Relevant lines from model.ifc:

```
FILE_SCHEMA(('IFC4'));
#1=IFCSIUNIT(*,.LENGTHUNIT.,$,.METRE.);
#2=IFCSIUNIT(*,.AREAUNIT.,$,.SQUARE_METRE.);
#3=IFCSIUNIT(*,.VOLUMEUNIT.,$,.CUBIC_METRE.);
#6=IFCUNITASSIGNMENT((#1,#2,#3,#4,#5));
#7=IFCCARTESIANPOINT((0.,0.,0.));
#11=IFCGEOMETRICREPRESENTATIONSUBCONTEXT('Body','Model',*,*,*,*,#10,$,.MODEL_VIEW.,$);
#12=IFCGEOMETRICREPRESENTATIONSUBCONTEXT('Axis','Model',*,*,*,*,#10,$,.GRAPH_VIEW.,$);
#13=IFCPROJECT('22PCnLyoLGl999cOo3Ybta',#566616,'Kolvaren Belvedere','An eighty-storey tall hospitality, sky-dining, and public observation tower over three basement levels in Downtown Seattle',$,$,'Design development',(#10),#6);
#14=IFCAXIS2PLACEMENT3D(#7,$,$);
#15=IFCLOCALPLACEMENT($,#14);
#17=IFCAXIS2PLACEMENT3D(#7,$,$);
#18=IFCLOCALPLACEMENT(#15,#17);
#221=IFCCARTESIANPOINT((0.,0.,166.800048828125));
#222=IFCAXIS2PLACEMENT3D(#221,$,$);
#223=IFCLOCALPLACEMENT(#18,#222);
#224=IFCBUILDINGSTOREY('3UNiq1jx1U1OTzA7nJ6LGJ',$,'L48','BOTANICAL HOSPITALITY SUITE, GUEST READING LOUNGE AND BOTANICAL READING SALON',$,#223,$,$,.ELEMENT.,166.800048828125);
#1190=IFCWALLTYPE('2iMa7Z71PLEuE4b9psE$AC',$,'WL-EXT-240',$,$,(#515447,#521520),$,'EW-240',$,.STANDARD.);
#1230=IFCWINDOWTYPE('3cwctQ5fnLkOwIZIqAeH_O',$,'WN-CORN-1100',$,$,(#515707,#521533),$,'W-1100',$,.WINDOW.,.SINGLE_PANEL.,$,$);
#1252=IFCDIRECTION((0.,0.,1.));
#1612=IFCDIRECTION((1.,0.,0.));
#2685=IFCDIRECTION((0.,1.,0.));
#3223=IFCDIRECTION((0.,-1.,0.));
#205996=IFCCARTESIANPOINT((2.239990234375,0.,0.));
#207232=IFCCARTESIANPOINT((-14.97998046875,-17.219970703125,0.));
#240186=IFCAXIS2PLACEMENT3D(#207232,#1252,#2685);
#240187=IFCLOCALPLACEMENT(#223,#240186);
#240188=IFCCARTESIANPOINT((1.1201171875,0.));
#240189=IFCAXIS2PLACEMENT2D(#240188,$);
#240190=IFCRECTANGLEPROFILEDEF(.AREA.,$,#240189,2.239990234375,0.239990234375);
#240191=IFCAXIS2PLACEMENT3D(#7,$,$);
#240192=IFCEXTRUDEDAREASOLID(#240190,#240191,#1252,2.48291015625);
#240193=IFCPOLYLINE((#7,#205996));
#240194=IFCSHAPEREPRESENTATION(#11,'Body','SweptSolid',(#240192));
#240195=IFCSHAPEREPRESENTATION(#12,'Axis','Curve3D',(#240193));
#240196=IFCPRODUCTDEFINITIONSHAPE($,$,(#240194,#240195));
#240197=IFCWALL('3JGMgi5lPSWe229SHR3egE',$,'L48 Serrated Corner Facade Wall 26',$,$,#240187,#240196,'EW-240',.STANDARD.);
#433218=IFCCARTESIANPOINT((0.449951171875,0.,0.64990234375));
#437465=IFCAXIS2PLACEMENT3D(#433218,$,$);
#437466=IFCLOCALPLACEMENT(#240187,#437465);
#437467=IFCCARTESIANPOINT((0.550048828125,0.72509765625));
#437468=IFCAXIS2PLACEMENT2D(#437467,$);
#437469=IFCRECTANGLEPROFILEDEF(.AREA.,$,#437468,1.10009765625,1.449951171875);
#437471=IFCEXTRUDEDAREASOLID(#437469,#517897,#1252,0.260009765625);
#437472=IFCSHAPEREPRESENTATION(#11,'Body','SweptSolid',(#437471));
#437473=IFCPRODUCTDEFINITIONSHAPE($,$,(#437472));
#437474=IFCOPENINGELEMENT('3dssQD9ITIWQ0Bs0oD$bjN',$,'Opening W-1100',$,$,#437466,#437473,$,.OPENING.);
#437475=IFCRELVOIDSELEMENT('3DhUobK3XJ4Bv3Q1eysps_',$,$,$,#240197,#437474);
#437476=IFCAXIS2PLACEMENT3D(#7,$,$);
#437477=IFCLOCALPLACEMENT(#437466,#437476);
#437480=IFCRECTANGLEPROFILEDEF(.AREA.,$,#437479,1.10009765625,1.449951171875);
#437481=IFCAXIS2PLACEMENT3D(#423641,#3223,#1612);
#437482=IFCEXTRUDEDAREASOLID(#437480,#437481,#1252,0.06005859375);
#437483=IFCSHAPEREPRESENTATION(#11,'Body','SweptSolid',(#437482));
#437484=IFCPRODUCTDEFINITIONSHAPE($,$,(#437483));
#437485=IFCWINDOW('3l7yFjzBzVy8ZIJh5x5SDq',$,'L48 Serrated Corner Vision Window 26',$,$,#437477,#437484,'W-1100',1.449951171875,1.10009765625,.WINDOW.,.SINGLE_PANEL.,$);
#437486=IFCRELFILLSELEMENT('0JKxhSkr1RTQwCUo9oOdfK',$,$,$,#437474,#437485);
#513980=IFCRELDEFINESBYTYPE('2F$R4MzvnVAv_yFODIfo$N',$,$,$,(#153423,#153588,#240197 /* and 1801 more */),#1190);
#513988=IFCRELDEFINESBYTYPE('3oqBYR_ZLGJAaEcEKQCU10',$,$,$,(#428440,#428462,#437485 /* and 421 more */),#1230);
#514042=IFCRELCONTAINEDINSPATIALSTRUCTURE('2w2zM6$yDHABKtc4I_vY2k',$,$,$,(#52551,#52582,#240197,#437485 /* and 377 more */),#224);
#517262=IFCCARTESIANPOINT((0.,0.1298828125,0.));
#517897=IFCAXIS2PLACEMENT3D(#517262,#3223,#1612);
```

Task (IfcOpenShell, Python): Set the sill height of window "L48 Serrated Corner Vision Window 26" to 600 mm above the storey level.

```python
import numpy as np
import ifcopenshell
import ifcopenshell.api.geometry
import ifcopenshell.geom
import ifcopenshell.util.element
import ifcopenshell.util.placement
import ifcopenshell.util.shape
import ifcopenshell.util.unit

model = ifcopenshell.open("model.ifc")
unit_scale = ifcopenshell.util.unit.calculate_unit_scale(model)

window = model.by_id(437485)
opening = window.FillsVoids[0].RelatingOpeningElement
storey = ifcopenshell.util.element.get_container(window, ifc_class="IfcBuildingStorey")
level = ifcopenshell.util.placement.get_local_placement(storey.ObjectPlacement)[2, 3]

# The opening's origin need not be at the sill, so measure its lowest point.
shape = ifcopenshell.geom.create_shape(ifcopenshell.geom.settings(), opening)
bottom = ifcopenshell.util.shape.get_shape_bottom_elevation(shape, shape.geometry) / unit_scale
dz = level + 0.6 - bottom

shift = np.array([0.0, 0.0, dz])
# The window is placed relative to its opening, so it follows when the opening moves.
matrix = ifcopenshell.util.placement.get_local_placement(opening.ObjectPlacement)
matrix[:3, 3] += shift
ifcopenshell.api.geometry.edit_object_placement(
    model, product=opening, matrix=matrix, is_si=False, should_transform_children=True
)

print(f"moved by {dz * unit_scale:+.3f} m")

model.write("model-out.ifc")
```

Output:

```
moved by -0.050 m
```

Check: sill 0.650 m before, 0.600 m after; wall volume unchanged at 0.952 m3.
